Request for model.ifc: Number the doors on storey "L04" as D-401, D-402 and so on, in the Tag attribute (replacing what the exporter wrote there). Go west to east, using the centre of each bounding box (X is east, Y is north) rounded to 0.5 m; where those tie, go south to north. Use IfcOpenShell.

First a look at what the model holds.

```python
import ifcopenshell
import ifcopenshell.util.element
import ifcopenshell.util.placement

model = ifcopenshell.open("model.ifc")
print(model.schema)
storey = next(s for s in model.by_type("IfcBuildingStorey") if s.Name == "L04")
doors = [e for e in ifcopenshell.util.element.get_decomposition(storey) if e.is_a("IfcDoor")]
for e in sorted(doors, key=lambda e: e.id()):
    origin = ifcopenshell.util.placement.get_local_placement(e.ObjectPlacement)[:3, 3]
    print(e.id(), e.Tag, e.Name, origin.round(2) + 0.0, sep=" | ")
```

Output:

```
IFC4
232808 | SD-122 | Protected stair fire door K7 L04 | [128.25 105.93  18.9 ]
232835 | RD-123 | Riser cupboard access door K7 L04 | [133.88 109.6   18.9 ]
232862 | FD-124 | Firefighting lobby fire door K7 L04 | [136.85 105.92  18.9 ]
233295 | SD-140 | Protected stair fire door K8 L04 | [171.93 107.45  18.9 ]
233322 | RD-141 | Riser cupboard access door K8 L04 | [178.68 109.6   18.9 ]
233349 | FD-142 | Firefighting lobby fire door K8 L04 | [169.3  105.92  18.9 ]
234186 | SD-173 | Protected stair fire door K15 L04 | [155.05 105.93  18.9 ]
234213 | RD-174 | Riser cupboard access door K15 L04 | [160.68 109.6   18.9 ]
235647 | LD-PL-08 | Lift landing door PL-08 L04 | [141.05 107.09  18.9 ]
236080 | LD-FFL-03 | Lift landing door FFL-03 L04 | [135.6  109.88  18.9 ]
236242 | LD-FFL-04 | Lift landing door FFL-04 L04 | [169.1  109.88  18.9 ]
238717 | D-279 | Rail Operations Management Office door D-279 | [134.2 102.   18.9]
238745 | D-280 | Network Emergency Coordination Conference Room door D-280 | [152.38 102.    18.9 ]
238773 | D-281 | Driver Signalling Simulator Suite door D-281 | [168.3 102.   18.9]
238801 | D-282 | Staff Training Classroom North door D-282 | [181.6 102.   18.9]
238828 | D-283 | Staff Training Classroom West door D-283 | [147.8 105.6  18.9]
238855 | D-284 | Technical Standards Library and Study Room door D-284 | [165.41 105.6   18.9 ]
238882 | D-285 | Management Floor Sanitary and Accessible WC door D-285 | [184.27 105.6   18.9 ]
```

```python
import ifcopenshell
import ifcopenshell.geom
import ifcopenshell.util.element
import ifcopenshell.util.shape

model = ifcopenshell.open("model.ifc")
settings = ifcopenshell.geom.settings()
settings.set("use-world-coords", True)


def centre(element):
    shape = ifcopenshell.geom.create_shape(settings, element)
    return ifcopenshell.util.shape.get_bbox_centroid(shape.geometry)


storey = next(s for s in model.by_type("IfcBuildingStorey") if s.Name == "L04")
doors = [e for e in ifcopenshell.util.element.get_decomposition(storey) if e.is_a("IfcDoor")]

# Insertion points can sit at a corner or the storey origin, so sort by the geometry (in metres).
centres = {e: centre(e) for e in doors}
doors.sort(key=lambda e: (round(centres[e][0] / 0.5), centres[e][1]))

for i, e in enumerate(doors, start=1):
    number = f"D-4{i:02d}"
    e.Tag = number
    print(e.id(), number)

model.write("model-out.ifc")
```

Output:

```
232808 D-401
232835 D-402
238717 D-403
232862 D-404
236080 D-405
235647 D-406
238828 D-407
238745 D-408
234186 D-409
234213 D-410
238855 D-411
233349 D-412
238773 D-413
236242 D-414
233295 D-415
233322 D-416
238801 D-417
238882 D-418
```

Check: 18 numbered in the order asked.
